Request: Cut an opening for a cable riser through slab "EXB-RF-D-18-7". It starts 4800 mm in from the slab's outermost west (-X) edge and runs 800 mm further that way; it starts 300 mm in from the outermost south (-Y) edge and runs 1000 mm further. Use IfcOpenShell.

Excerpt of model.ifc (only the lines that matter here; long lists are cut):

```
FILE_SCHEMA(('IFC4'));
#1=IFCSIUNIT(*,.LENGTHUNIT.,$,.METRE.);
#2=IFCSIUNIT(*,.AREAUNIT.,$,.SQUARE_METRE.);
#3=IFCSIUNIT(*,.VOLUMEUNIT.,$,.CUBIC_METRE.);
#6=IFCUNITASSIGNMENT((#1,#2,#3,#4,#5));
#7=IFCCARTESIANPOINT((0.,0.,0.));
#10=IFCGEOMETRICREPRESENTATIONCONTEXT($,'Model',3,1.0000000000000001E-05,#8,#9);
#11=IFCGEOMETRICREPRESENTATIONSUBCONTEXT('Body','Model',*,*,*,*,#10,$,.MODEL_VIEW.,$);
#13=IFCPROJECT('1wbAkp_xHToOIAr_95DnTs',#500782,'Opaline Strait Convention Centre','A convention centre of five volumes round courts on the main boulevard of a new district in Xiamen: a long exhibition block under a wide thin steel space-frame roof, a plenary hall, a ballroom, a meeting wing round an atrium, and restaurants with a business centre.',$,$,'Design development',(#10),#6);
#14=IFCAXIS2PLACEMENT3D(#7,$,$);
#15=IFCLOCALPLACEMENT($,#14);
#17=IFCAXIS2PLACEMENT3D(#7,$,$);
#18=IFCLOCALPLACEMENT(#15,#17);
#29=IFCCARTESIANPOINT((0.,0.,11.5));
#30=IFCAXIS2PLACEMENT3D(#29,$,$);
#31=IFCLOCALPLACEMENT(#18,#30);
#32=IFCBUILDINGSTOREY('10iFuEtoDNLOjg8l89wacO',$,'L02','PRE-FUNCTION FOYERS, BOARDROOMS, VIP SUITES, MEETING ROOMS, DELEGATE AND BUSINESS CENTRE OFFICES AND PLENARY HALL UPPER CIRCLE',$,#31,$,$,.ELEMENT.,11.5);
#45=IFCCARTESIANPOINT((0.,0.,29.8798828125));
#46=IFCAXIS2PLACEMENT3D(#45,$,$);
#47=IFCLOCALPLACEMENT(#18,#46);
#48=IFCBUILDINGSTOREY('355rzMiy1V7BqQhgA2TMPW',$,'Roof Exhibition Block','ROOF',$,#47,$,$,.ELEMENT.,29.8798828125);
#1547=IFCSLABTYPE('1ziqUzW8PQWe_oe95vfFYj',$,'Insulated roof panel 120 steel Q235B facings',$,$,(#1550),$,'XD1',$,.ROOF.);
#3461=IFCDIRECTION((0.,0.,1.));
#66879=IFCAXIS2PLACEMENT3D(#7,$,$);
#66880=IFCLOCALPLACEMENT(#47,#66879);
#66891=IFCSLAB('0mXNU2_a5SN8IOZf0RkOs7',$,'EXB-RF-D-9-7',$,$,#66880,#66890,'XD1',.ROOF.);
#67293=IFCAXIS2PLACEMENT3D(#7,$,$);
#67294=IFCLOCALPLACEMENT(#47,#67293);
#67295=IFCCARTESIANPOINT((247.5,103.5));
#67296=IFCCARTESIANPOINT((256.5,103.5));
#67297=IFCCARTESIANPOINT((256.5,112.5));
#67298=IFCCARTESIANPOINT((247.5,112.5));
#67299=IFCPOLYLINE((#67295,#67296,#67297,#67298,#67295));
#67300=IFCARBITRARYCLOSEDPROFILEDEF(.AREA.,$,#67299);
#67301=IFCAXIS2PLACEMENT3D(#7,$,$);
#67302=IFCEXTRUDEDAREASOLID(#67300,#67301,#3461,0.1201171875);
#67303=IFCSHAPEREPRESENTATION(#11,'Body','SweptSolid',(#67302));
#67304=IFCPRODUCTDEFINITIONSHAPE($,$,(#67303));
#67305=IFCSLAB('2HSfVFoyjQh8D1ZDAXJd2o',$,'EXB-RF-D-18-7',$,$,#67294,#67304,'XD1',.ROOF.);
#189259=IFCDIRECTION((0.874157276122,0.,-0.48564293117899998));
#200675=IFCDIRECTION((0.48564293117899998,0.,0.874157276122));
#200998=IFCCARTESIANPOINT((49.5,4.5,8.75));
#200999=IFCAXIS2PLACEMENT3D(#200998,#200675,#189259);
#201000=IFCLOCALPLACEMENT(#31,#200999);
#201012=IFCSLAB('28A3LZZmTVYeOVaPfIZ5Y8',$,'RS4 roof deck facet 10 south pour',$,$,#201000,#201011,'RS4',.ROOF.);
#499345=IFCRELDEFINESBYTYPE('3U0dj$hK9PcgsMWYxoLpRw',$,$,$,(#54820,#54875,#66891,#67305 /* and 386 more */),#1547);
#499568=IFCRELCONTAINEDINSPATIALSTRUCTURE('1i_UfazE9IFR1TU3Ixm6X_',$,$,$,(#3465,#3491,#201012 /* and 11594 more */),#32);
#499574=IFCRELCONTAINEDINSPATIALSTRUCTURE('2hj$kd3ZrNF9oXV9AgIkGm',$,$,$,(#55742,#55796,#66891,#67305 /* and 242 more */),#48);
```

```python
import numpy as np
import ifcopenshell
import ifcopenshell.api.feature
import ifcopenshell.api.geometry
import ifcopenshell.api.root
import ifcopenshell.geom
import ifcopenshell.util.placement
import ifcopenshell.util.representation
import ifcopenshell.util.shape
import ifcopenshell.util.unit

model = ifcopenshell.open("model.ifc")
unit_scale = ifcopenshell.util.unit.calculate_unit_scale(model)
settings = ifcopenshell.geom.settings()


def volume(element):
    """Net volume in cubic metres, openings subtracted."""
    shape = ifcopenshell.geom.create_shape(settings, element)
    return ifcopenshell.util.shape.get_volume(shape.geometry)


slab = model.by_guid("2HSfVFoyjQh8D1ZDAXJd2o")
before = volume(slab)

# Extent in the slab's own axes, in metres. The edges named are its -X and -Y sides.
slab_shape = ifcopenshell.geom.create_shape(settings, slab)
vertices = ifcopenshell.util.shape.get_vertices(slab_shape.geometry)
x_min, y_min, bottom = vertices.min(axis=0)
top = vertices[:, 2].max()

opening = ifcopenshell.api.root.create_entity(model, ifc_class="IfcOpeningElement", name="Cable riser opening", predefined_type="OPENING")
context = ifcopenshell.util.representation.get_context(model, "Model", "Body", "MODEL_VIEW")
width, depth = 0.8, 1
outline = [(0.0, 0.0), (width, 0.0), (width, depth), (0.0, depth), (0.0, 0.0)]
# Overshoot both faces by 50 mm so the cut is clean.
shape = ifcopenshell.api.geometry.add_slab_representation(
    model, context=context, depth=top - bottom + 0.1, polyline=outline
)
ifcopenshell.api.geometry.assign_representation(model, product=opening, representation=shape)

matrix = ifcopenshell.util.placement.get_local_placement(slab.ObjectPlacement)
matrix[:, 3] = matrix @ np.append(np.array([x_min + 4.8, y_min + 0.3, bottom - 0.05]) / unit_scale, 1.0)
ifcopenshell.api.geometry.edit_object_placement(model, product=opening, matrix=matrix, is_si=False)
ifcopenshell.api.feature.add_feature(model, feature=opening, element=slab)

after = volume(slab)

print(f"slab volume {before:.3f} -> {after:.3f} m3")

model.write("model_updated.ifc")
```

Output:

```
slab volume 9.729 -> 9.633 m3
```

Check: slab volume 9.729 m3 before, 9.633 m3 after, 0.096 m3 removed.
